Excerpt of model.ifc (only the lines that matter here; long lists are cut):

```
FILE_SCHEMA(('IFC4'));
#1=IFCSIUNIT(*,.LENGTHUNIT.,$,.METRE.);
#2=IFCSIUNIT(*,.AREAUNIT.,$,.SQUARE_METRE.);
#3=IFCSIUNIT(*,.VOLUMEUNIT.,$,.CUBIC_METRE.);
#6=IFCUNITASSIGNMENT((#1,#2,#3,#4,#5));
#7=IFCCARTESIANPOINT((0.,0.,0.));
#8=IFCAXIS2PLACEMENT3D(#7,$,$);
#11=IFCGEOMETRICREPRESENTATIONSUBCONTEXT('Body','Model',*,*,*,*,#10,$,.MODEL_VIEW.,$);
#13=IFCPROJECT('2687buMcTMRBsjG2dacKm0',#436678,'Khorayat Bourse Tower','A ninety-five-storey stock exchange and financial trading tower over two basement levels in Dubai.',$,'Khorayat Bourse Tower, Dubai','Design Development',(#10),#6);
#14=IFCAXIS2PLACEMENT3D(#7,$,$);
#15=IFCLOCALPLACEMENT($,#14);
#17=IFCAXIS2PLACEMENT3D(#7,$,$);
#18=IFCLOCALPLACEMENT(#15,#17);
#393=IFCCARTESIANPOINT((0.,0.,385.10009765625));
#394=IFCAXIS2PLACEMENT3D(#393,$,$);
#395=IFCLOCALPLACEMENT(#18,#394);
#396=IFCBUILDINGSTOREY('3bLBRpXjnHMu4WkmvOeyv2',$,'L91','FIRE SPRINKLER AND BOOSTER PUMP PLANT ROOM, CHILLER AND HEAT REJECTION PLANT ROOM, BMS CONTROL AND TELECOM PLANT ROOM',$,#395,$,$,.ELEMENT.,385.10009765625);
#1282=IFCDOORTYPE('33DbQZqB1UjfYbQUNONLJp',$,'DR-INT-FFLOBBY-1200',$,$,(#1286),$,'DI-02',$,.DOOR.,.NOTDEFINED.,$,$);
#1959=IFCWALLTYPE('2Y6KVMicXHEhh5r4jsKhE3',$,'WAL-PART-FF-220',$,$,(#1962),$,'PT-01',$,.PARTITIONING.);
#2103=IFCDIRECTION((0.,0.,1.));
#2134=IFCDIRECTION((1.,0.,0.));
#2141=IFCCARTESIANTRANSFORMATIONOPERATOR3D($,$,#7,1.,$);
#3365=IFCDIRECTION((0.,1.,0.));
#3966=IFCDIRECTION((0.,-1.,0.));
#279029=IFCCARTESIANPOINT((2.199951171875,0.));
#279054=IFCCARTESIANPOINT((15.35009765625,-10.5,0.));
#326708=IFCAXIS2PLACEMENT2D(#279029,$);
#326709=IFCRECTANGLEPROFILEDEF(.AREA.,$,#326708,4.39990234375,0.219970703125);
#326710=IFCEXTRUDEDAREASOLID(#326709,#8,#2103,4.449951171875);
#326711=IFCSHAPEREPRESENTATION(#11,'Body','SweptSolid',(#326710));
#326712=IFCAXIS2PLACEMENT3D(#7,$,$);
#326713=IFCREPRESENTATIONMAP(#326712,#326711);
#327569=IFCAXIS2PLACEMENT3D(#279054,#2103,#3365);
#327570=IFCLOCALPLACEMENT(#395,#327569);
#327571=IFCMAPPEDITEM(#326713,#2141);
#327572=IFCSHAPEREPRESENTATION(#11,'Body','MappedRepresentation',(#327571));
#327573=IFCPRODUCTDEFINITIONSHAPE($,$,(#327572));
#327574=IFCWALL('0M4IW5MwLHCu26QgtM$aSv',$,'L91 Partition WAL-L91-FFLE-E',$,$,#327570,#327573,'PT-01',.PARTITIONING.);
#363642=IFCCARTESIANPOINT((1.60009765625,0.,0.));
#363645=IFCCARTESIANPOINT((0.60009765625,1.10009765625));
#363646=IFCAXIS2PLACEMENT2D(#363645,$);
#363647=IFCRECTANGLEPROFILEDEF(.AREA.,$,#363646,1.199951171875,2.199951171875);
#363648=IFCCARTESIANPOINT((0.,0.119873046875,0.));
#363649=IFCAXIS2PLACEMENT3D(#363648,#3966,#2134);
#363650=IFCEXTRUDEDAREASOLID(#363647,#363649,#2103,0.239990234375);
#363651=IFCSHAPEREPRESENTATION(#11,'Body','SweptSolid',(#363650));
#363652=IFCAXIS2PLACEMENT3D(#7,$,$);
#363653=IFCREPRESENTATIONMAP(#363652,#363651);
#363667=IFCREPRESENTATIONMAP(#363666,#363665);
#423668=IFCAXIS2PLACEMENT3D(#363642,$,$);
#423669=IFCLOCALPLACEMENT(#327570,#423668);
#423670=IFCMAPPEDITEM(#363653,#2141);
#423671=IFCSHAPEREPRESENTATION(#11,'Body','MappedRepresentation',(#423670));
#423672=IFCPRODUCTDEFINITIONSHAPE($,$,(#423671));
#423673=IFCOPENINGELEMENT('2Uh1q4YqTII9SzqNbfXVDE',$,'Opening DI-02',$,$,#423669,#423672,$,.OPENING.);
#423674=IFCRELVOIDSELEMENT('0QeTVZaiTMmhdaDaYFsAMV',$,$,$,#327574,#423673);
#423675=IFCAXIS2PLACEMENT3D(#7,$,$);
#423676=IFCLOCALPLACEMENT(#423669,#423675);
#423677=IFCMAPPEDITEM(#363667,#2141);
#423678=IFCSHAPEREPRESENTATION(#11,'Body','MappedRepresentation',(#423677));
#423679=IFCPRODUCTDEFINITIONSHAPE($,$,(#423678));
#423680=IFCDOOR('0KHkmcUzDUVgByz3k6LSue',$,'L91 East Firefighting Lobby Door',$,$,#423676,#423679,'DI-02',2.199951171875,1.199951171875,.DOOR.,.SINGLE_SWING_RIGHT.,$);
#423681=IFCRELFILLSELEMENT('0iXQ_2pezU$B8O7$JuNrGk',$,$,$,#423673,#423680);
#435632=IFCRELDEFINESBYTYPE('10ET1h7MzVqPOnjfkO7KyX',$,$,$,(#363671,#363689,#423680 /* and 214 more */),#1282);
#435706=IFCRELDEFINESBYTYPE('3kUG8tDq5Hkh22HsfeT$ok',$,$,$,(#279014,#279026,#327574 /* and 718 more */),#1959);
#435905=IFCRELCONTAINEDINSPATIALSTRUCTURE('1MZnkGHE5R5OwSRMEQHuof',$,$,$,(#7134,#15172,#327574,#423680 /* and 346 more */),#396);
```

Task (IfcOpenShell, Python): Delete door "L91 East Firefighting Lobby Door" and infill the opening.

```python
import ifcopenshell
import ifcopenshell.api.feature
import ifcopenshell.api.root
import ifcopenshell.geom
import ifcopenshell.util.shape

model = ifcopenshell.open("model.ifc")
settings = ifcopenshell.geom.settings()


def volume(element):
    """Net volume in cubic metres, openings subtracted."""
    shape = ifcopenshell.geom.create_shape(settings, element)
    return ifcopenshell.util.shape.get_volume(shape.geometry)


door = model.by_guid("0KHkmcUzDUVgByz3k6LSue")
opening = door.FillsVoids[0].RelatingOpeningElement
wall = opening.VoidsElements[0].RelatingBuildingElement
before = volume(wall)

ifcopenshell.api.root.remove_product(model, product=door)
ifcopenshell.api.feature.remove_feature(model, feature=opening)

after = volume(wall)

print(f"wall volume {before:.3f} -> {after:.3f} m3")

model.write("model_updated.ifc")
```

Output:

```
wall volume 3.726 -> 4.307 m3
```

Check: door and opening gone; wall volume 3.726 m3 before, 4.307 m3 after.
